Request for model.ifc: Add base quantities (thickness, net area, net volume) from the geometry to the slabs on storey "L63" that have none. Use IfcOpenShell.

First a look at what the model holds.

```python
import ifcopenshell
import ifcopenshell.util.element
import ifcopenshell.util.unit

model = ifcopenshell.open("model.ifc")
print(model.schema)
for unit_type in ("LENGTHUNIT", "AREAUNIT", "VOLUMEUNIT"):
    print(unit_type, ifcopenshell.util.unit.calculate_unit_scale(model, unit_type))
storey = next(s for s in model.by_type("IfcBuildingStorey") if s.Name == "L63")
slabs = [e for e in ifcopenshell.util.element.get_decomposition(storey) if e.is_a("IfcSlab")]
for e in sorted(slabs, key=lambda e: e.id()):
    print(e.id(), e.is_a(), e.Name, list(ifcopenshell.util.element.get_psets(e, qtos_only=True)), sep=" | ")
```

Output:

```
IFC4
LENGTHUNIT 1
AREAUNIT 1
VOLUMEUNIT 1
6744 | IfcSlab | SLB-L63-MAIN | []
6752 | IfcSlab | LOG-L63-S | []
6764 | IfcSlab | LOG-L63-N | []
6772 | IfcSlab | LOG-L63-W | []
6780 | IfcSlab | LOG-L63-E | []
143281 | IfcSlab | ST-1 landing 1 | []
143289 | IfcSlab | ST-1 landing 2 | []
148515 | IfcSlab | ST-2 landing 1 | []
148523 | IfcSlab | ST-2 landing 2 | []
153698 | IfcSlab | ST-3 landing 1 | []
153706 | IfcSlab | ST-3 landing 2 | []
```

```python
import ifcopenshell
import ifcopenshell.api.pset
import ifcopenshell.geom
import ifcopenshell.util.element
import ifcopenshell.util.shape
import ifcopenshell.util.unit

model = ifcopenshell.open("model.ifc")
unit_scale = ifcopenshell.util.unit.calculate_unit_scale(model)
area_scale = ifcopenshell.util.unit.calculate_unit_scale(model, "AREAUNIT")
volume_scale = ifcopenshell.util.unit.calculate_unit_scale(model, "VOLUMEUNIT")
settings = ifcopenshell.geom.settings()

storey = next(s for s in model.by_type("IfcBuildingStorey") if s.Name == "L63")
slabs = [e for e in ifcopenshell.util.element.get_decomposition(storey) if e.is_a("IfcSlab")]

for e in sorted(slabs, key=lambda e: e.id()):
    if ifcopenshell.util.element.get_psets(e, qtos_only=True, should_inherit=False):
        continue
    # Geometry comes back in metres, in the element's own axes.
    shape = ifcopenshell.geom.create_shape(settings, e)
    values = {
        "Width": ifcopenshell.util.shape.get_z(shape.geometry) / unit_scale,
        "NetArea": ifcopenshell.util.shape.get_footprint_area(shape.geometry) / area_scale,
        "NetVolume": ifcopenshell.util.shape.get_volume(shape.geometry) / volume_scale,
    }
    qto = ifcopenshell.api.pset.add_qto(model, product=e, name="Qto_SlabBaseQuantities")
    ifcopenshell.api.pset.edit_qto(model, qto=qto, properties=values)
    print(e.id(), {k: round(v, 3) for k, v in values.items()})

model.write("model-out.ifc")
```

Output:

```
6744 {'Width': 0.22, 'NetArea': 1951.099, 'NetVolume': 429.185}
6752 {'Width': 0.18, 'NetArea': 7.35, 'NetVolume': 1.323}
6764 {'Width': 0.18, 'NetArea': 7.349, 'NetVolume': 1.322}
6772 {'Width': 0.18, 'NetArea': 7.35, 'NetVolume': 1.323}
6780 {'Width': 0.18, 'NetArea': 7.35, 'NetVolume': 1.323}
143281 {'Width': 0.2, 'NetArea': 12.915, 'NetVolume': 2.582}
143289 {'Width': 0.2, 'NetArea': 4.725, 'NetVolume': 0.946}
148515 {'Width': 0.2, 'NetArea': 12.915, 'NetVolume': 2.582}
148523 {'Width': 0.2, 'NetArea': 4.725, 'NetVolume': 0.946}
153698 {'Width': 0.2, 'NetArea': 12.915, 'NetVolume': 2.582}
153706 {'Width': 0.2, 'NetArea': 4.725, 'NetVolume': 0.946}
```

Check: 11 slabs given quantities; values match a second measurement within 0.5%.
